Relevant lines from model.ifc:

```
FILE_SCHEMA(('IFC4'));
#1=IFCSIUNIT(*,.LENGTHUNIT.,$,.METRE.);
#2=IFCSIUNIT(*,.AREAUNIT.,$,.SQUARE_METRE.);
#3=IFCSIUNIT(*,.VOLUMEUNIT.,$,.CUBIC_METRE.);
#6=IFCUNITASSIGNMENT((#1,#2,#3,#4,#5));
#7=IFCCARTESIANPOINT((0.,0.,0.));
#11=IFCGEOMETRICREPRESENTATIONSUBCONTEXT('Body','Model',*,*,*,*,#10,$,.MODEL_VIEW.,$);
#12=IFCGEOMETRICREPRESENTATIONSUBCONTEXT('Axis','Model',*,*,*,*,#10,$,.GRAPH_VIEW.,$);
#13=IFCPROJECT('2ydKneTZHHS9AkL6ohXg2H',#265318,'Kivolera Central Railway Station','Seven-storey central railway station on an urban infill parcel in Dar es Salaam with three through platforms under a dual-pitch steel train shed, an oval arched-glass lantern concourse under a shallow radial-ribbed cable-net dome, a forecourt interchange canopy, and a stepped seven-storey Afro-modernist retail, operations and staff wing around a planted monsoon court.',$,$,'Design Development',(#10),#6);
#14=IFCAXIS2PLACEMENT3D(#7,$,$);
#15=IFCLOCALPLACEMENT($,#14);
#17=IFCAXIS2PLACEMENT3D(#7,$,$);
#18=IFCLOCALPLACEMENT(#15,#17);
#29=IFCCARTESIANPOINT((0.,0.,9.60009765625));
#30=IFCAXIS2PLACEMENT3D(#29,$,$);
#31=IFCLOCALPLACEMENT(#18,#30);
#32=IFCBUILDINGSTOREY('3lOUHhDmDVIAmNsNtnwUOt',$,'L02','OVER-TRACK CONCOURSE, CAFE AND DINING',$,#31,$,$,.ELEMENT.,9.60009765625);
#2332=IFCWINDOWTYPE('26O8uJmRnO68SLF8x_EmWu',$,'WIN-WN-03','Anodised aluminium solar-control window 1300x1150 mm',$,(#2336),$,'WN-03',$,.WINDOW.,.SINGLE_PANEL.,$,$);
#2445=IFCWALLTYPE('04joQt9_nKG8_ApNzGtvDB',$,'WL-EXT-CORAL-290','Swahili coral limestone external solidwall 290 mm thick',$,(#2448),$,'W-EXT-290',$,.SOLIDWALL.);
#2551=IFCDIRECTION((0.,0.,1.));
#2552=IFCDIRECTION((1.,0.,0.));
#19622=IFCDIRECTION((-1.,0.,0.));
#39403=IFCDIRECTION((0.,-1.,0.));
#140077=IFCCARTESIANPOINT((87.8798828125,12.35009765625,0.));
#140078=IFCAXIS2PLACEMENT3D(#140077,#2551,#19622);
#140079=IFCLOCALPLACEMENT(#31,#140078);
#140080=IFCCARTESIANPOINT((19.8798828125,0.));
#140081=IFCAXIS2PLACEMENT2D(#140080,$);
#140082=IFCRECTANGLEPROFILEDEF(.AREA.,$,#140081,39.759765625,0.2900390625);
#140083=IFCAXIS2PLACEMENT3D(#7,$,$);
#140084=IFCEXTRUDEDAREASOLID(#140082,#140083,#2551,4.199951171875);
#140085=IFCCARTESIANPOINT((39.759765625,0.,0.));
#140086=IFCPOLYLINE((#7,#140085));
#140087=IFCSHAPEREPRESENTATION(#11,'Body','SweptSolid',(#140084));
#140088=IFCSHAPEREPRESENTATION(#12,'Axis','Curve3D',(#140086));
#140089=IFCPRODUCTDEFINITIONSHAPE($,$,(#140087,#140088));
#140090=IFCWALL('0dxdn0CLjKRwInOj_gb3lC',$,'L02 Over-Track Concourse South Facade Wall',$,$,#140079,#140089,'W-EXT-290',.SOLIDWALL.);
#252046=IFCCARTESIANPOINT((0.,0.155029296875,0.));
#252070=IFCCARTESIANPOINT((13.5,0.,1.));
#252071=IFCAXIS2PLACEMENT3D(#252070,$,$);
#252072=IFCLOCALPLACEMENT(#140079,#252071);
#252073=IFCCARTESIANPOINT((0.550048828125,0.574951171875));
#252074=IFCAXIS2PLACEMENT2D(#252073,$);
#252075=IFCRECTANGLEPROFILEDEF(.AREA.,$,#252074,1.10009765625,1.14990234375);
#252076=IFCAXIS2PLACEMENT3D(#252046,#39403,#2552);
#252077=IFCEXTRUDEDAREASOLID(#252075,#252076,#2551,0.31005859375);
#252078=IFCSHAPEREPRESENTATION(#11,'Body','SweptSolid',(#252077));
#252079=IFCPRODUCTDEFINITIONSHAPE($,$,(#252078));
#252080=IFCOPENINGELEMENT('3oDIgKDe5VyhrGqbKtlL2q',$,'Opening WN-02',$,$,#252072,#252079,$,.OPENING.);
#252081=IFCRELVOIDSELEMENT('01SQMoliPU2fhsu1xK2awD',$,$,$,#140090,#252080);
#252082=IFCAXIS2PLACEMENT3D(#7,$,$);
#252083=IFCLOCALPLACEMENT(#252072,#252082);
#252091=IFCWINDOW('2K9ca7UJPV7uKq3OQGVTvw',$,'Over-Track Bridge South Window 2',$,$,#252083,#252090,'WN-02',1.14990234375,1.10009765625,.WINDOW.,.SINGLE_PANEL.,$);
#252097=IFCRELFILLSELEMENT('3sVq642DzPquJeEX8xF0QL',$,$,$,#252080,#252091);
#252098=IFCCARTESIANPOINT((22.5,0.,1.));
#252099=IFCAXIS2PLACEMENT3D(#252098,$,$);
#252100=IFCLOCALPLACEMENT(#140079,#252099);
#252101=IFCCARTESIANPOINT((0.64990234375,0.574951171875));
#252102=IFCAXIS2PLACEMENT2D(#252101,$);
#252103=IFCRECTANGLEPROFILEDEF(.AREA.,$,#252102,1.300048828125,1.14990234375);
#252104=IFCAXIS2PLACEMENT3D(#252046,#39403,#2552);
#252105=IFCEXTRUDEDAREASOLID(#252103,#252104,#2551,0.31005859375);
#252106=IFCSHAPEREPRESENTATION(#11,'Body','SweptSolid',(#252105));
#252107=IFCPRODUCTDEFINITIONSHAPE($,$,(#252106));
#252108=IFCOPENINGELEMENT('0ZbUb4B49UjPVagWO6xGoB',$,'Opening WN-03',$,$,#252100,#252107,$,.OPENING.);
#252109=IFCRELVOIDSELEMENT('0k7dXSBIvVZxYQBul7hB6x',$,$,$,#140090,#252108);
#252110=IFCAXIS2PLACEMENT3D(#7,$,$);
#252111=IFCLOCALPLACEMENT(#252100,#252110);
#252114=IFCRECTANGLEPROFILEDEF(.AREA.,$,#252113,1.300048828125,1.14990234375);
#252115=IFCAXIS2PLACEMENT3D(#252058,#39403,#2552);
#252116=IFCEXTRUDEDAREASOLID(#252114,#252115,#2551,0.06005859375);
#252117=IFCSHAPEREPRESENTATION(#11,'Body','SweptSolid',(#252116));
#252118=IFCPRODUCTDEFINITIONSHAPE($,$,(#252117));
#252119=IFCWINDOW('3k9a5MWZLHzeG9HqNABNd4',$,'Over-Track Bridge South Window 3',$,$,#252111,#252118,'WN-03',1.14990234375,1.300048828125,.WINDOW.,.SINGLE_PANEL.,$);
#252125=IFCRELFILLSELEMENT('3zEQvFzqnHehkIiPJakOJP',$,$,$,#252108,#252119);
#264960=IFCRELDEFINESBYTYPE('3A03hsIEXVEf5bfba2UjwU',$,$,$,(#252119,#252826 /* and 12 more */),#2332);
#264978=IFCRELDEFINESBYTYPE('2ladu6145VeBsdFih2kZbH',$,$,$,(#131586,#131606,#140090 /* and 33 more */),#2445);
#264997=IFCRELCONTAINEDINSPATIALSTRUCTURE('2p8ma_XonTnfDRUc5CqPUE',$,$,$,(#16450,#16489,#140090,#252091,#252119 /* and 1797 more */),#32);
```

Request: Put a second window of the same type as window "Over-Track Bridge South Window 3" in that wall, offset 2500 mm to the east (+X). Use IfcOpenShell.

```python
import ifcopenshell
import ifcopenshell.api.feature
import ifcopenshell.api.geometry
import ifcopenshell.api.root
import ifcopenshell.geom
import ifcopenshell.util.element
import ifcopenshell.util.placement
import ifcopenshell.util.shape
import ifcopenshell.util.unit

model = ifcopenshell.open("model.ifc")
unit_scale = ifcopenshell.util.unit.calculate_unit_scale(model)
settings = ifcopenshell.geom.settings()


def volume(element):
    """Net volume in cubic metres, openings subtracted."""
    shape = ifcopenshell.geom.create_shape(settings, element)
    return ifcopenshell.util.shape.get_volume(shape.geometry)


window = model.by_guid("3k9a5MWZLHzeG9HqNABNd4")
opening = window.FillsVoids[0].RelatingOpeningElement
wall = opening.VoidsElements[0].RelatingBuildingElement
before = volume(wall)
shift = ifcopenshell.util.placement.get_local_placement(wall.ObjectPlacement)[:3, 0] * -2.5 / unit_scale

# copy_class copies the void relationship, type, container and properties, but no geometry.
new_opening = ifcopenshell.api.root.copy_class(model, product=opening)
new_opening.Representation = ifcopenshell.util.element.copy_deep(
    model, opening.Representation, exclude=["IfcGeometricRepresentationContext", "IfcRepresentationMap"]
)
new_window = ifcopenshell.api.root.copy_class(model, product=window)
new_window.Representation = ifcopenshell.util.element.copy_deep(
    model, window.Representation, exclude=["IfcGeometricRepresentationContext", "IfcRepresentationMap"]
)
new_window.Tag = None
ifcopenshell.api.feature.add_filling(model, opening=new_opening, element=new_window)

for old, new in ((opening, new_opening), (window, new_window)):
    matrix = ifcopenshell.util.placement.get_local_placement(old.ObjectPlacement)
    matrix[:3, 3] += shift
    ifcopenshell.api.geometry.edit_object_placement(model, product=new, matrix=matrix, is_si=False)

after = volume(wall)

print(f"wall volume {before:.3f} -> {after:.3f} m3")

model.write("model_rev.ifc")
```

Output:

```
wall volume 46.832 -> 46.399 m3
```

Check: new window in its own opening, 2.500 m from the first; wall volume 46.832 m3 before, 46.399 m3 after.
